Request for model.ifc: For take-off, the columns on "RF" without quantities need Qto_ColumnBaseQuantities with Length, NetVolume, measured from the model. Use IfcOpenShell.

First a look at what the model holds.

```python
import ifcopenshell
import ifcopenshell.util.element
import ifcopenshell.util.unit

model = ifcopenshell.open("model.ifc")
print(model.schema)
for unit_type in ("LENGTHUNIT", "AREAUNIT", "VOLUMEUNIT"):
    print(unit_type, ifcopenshell.util.unit.calculate_unit_scale(model, unit_type))
storey = next(s for s in model.by_type("IfcBuildingStorey") if s.Name == "RF")
columns = [e for e in ifcopenshell.util.element.get_decomposition(storey) if e.is_a("IfcColumn")]
for e in sorted(columns, key=lambda e: e.id()):
    print(e.id(), e.is_a(), e.Name, list(ifcopenshell.util.element.get_psets(e, qtos_only=True)), sep=" | ")
```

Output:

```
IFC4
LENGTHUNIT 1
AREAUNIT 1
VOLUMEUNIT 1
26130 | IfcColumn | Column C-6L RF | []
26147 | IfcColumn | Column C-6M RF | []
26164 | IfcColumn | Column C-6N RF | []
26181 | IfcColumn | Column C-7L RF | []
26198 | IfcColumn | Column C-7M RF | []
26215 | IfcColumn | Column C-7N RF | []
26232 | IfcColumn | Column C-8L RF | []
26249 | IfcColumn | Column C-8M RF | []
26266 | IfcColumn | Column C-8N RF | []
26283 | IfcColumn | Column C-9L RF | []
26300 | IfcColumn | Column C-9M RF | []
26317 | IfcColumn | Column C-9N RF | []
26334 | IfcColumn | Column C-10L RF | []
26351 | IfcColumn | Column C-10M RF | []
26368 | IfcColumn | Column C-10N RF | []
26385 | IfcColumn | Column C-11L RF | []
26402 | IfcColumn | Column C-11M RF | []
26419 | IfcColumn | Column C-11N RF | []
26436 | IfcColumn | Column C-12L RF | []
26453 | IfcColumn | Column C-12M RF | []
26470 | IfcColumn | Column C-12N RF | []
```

```python
import ifcopenshell
import ifcopenshell.api.pset
import ifcopenshell.geom
import ifcopenshell.util.element
import ifcopenshell.util.shape
import ifcopenshell.util.unit

model = ifcopenshell.open("model.ifc")
unit_scale = ifcopenshell.util.unit.calculate_unit_scale(model)
volume_scale = ifcopenshell.util.unit.calculate_unit_scale(model, "VOLUMEUNIT")
settings = ifcopenshell.geom.settings()

storey = next(s for s in model.by_type("IfcBuildingStorey") if s.Name == "RF")
columns = [e for e in ifcopenshell.util.element.get_decomposition(storey) if e.is_a("IfcColumn")]

for e in sorted(columns, key=lambda e: e.id()):
    if ifcopenshell.util.element.get_psets(e, qtos_only=True, should_inherit=False):
        continue
    # Geometry comes back in metres, in the element's own axes.
    shape = ifcopenshell.geom.create_shape(settings, e)
    values = {
        "Length": ifcopenshell.util.shape.get_z(shape.geometry) / unit_scale,
        "NetVolume": ifcopenshell.util.shape.get_volume(shape.geometry) / volume_scale,
    }
    qto = ifcopenshell.api.pset.add_qto(model, product=e, name="Qto_ColumnBaseQuantities")
    ifcopenshell.api.pset.edit_qto(model, qto=qto, properties=values)
    print(e.id(), {k: round(v, 3) for k, v in values.items()})

model.write("model_updated.ifc")
```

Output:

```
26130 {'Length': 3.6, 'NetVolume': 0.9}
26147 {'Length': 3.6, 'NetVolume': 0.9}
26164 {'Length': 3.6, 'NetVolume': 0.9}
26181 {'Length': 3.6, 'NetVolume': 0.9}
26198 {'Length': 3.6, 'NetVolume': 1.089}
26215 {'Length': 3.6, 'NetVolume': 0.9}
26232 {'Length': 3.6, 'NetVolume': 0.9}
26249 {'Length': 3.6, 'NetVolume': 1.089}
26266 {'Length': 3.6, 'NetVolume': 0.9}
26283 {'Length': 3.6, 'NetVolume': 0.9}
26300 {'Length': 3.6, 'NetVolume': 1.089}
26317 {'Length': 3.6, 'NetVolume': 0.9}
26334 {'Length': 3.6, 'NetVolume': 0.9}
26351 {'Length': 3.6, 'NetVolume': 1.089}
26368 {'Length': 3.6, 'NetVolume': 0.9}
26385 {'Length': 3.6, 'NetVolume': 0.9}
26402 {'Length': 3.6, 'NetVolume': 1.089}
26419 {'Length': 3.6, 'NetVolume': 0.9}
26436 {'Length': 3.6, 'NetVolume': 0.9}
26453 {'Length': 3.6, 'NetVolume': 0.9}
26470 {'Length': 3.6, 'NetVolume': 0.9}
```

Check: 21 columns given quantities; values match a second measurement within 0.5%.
